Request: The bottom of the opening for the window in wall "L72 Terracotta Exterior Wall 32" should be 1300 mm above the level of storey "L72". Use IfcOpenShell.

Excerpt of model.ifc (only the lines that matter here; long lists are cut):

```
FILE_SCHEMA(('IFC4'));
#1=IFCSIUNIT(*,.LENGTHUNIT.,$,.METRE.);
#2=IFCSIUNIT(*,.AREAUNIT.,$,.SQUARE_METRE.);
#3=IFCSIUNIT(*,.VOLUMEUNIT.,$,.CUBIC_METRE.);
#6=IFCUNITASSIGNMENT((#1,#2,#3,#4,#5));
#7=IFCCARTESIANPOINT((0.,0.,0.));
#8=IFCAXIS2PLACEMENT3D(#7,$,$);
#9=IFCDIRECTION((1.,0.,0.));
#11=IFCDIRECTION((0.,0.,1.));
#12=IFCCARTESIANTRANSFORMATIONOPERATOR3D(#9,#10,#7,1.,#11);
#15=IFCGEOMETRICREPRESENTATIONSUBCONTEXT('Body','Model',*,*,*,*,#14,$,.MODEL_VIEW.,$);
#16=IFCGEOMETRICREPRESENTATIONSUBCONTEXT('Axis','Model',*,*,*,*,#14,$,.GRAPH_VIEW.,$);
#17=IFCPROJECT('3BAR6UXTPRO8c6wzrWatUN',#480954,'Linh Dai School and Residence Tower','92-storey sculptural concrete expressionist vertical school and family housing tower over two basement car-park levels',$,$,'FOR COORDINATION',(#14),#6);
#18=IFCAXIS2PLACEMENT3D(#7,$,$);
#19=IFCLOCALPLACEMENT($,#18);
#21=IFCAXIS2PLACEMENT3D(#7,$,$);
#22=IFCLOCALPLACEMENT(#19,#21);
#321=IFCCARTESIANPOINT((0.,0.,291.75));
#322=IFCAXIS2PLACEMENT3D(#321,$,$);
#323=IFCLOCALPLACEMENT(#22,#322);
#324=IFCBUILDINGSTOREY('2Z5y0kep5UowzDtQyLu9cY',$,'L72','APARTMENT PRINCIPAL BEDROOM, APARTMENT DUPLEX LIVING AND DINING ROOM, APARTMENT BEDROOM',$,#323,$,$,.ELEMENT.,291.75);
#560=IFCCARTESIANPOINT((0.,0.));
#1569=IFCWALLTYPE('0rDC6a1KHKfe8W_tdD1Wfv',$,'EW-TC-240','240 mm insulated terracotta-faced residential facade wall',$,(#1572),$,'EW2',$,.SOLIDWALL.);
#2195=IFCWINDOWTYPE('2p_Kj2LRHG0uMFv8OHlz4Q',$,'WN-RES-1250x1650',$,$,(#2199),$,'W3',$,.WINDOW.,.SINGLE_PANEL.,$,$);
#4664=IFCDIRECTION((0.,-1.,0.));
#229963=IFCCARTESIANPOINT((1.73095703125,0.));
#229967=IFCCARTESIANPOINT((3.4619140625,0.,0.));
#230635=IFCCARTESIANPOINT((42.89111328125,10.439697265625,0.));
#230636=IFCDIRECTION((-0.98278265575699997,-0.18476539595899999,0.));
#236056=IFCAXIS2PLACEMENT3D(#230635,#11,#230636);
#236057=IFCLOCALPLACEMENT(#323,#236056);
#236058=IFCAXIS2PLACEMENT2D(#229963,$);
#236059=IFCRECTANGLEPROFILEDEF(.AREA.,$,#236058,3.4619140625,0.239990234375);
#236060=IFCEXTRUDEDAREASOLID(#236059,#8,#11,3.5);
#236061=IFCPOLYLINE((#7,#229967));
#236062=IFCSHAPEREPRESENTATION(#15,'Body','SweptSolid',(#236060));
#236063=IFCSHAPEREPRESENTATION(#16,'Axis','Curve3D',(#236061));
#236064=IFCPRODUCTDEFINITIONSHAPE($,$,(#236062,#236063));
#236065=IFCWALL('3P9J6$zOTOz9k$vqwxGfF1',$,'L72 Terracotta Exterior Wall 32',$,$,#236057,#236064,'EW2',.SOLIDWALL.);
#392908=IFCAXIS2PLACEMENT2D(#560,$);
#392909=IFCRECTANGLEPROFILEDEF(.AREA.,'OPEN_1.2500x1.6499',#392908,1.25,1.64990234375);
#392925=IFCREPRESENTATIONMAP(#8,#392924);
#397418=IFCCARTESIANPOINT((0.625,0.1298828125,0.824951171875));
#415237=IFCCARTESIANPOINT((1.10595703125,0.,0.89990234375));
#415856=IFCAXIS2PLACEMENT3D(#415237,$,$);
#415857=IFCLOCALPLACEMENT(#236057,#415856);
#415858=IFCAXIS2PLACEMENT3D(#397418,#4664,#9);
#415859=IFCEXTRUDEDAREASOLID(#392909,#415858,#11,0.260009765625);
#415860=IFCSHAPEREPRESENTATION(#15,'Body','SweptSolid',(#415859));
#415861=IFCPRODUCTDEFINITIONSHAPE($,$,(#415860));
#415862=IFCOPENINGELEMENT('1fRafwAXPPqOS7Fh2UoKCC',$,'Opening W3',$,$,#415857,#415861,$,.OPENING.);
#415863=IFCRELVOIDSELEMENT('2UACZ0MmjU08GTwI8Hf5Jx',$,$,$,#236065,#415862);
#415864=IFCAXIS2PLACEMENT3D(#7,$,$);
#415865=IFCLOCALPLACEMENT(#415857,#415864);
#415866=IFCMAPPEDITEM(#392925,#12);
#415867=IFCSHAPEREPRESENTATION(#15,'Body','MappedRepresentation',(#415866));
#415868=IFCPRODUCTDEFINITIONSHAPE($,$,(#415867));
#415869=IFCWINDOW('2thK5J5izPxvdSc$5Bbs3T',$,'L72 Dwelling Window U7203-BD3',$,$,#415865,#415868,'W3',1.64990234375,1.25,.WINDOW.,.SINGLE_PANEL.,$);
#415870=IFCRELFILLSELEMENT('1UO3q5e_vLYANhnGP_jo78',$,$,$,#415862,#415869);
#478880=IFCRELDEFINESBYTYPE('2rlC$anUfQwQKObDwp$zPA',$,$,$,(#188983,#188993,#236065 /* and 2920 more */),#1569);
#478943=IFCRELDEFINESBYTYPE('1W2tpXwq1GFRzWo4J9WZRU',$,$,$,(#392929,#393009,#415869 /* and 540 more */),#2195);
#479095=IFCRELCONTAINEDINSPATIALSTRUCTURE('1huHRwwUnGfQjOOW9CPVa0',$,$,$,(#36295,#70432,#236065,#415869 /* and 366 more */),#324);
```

```python
import numpy as np
import ifcopenshell
import ifcopenshell.api.geometry
import ifcopenshell.geom
import ifcopenshell.util.element
import ifcopenshell.util.placement
import ifcopenshell.util.shape
import ifcopenshell.util.unit

model = ifcopenshell.open("model.ifc")
unit_scale = ifcopenshell.util.unit.calculate_unit_scale(model)

window = model.by_guid("2thK5J5izPxvdSc$5Bbs3T")
opening = window.FillsVoids[0].RelatingOpeningElement
storey = ifcopenshell.util.element.get_container(window, ifc_class="IfcBuildingStorey")
level = ifcopenshell.util.placement.get_local_placement(storey.ObjectPlacement)[2, 3]

# The opening's origin need not be at the sill, so measure its lowest point.
shape = ifcopenshell.geom.create_shape(ifcopenshell.geom.settings(), opening)
bottom = ifcopenshell.util.shape.get_shape_bottom_elevation(shape, shape.geometry) / unit_scale
dz = level + 1.3 / unit_scale - bottom

shift = np.array([0.0, 0.0, dz])
# The window is placed relative to its opening, so it follows when the opening moves.
matrix = ifcopenshell.util.placement.get_local_placement(opening.ObjectPlacement)
matrix[:3, 3] += shift
ifcopenshell.api.geometry.edit_object_placement(
    model, product=opening, matrix=matrix, is_si=False, should_transform_children=True
)

print(f"moved by {dz * unit_scale:+.3f} m")

model.write("model-out.ifc")
```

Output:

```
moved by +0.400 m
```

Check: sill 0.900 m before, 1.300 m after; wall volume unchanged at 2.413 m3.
